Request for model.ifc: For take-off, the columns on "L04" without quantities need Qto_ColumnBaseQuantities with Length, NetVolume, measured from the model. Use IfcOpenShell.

First a look at what the model holds.

```python
import ifcopenshell
import ifcopenshell.util.element
import ifcopenshell.util.unit

model = ifcopenshell.open("model.ifc")
print(model.schema)
for unit_type in ("LENGTHUNIT", "AREAUNIT", "VOLUMEUNIT"):
    print(unit_type, ifcopenshell.util.unit.calculate_unit_scale(model, unit_type))
storey = next(s for s in model.by_type("IfcBuildingStorey") if s.Name == "L04")
columns = [e for e in ifcopenshell.util.element.get_decomposition(storey) if e.is_a("IfcColumn")]
for e in sorted(columns, key=lambda e: e.id()):
    print(e.id(), e.is_a(), e.Name, list(ifcopenshell.util.element.get_psets(e, qtos_only=True)), sep=" | ")
```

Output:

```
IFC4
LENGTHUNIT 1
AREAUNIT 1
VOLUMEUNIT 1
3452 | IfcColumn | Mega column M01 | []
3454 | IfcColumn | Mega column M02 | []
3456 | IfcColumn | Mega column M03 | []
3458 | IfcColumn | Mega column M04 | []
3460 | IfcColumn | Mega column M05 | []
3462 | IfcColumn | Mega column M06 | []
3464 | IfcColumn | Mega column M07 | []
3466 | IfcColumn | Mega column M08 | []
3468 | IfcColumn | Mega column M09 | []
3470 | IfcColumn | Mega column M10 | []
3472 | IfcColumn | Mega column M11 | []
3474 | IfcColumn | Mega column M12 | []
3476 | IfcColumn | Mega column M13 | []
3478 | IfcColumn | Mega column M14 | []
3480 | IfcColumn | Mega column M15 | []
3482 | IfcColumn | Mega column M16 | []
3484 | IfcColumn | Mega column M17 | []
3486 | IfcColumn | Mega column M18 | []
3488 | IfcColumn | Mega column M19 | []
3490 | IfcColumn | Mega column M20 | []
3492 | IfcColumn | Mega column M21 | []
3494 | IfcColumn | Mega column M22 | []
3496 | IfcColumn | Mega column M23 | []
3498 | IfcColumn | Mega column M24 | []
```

```python
import ifcopenshell
import ifcopenshell.api.pset
import ifcopenshell.geom
import ifcopenshell.util.element
import ifcopenshell.util.shape
import ifcopenshell.util.unit

model = ifcopenshell.open("model.ifc")
unit_scale = ifcopenshell.util.unit.calculate_unit_scale(model)
volume_scale = ifcopenshell.util.unit.calculate_unit_scale(model, "VOLUMEUNIT")
settings = ifcopenshell.geom.settings()

storey = next(s for s in model.by_type("IfcBuildingStorey") if s.Name == "L04")
columns = [e for e in ifcopenshell.util.element.get_decomposition(storey) if e.is_a("IfcColumn")]

for e in sorted(columns, key=lambda e: e.id()):
    if ifcopenshell.util.element.get_psets(e, qtos_only=True, should_inherit=False):
        continue
    # Geometry comes back in metres, in the element's own axes.
    shape = ifcopenshell.geom.create_shape(settings, e)
    values = {
        "Length": ifcopenshell.util.shape.get_z(shape.geometry) / unit_scale,
        "NetVolume": ifcopenshell.util.shape.get_volume(shape.geometry) / volume_scale,
    }
    qto = ifcopenshell.api.pset.add_qto(model, product=e, name="Qto_ColumnBaseQuantities")
    ifcopenshell.api.pset.edit_qto(model, qto=qto, properties=values)
    print(e.id(), {k: round(v, 3) for k, v in values.items()})

model.write("model-out.ifc")
```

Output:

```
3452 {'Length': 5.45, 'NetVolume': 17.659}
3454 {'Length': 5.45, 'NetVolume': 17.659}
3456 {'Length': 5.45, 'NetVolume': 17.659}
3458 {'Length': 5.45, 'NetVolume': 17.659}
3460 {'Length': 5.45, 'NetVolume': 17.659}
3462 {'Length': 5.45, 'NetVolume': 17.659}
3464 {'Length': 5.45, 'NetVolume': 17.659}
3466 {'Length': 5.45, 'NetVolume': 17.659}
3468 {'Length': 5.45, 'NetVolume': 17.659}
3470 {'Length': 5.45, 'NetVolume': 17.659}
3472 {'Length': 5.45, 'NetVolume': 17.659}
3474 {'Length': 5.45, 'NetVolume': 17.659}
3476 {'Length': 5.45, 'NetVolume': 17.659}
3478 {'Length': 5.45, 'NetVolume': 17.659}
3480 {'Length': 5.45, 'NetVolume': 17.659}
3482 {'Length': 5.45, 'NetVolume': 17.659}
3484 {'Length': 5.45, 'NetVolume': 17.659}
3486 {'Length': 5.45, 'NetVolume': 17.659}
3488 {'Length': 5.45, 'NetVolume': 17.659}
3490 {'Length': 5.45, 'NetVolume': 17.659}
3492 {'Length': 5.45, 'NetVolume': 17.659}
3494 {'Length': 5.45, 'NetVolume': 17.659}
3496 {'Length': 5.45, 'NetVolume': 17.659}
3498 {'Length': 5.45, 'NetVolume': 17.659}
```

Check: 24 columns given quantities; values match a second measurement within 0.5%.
